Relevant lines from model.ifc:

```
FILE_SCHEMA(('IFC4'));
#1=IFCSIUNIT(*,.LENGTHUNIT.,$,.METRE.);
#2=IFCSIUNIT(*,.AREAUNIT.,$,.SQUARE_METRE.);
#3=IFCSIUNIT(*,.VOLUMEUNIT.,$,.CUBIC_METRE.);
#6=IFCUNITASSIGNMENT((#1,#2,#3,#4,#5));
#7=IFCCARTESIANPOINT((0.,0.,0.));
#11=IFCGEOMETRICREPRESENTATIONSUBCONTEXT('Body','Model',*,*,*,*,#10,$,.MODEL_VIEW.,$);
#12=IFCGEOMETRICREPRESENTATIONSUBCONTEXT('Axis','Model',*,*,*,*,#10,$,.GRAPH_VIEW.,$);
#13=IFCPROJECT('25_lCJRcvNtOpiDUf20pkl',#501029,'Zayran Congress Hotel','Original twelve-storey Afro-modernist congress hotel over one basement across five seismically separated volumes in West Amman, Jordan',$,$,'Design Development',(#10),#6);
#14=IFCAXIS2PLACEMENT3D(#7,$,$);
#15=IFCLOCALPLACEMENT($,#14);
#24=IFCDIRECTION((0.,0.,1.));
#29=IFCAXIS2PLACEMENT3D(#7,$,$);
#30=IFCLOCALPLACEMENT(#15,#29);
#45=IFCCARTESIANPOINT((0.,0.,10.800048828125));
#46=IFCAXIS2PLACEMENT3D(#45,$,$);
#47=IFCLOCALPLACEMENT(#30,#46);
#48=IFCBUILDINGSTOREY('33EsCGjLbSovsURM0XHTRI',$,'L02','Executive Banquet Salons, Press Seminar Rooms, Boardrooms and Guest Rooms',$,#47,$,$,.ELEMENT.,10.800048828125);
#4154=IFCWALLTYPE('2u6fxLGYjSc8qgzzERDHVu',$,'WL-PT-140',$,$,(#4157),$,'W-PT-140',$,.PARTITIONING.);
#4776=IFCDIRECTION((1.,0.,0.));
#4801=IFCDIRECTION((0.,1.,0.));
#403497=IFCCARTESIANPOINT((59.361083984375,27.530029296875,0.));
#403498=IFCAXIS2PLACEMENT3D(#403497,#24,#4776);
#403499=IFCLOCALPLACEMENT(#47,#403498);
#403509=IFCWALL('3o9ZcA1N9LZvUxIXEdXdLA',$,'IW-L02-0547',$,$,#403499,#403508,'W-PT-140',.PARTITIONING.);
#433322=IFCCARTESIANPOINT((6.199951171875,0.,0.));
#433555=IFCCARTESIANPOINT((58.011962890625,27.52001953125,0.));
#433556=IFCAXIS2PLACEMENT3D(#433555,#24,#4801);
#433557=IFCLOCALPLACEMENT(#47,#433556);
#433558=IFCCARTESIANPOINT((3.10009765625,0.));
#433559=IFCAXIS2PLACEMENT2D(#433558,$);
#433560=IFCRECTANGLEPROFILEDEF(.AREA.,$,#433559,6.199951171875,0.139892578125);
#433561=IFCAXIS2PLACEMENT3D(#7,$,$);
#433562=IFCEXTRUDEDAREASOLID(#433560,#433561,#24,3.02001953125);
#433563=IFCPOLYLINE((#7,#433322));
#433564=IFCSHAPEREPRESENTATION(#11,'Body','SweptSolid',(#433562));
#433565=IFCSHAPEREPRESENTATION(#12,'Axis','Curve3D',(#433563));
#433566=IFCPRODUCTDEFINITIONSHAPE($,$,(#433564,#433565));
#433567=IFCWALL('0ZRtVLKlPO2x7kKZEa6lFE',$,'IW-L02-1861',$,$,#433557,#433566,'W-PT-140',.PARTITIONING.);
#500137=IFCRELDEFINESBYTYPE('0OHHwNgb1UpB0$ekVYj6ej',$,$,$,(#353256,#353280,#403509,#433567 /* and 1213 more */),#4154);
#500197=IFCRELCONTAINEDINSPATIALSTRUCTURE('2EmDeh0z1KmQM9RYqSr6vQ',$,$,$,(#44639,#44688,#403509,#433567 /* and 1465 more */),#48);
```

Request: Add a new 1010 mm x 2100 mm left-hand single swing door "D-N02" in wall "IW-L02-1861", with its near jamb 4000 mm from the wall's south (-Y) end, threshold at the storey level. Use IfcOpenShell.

```python
import numpy as np
import ifcopenshell
import ifcopenshell.api.feature
import ifcopenshell.api.geometry
import ifcopenshell.api.root
import ifcopenshell.api.spatial
import ifcopenshell.geom
import ifcopenshell.util.element
import ifcopenshell.util.placement
import ifcopenshell.util.representation
import ifcopenshell.util.shape
import ifcopenshell.util.unit

model = ifcopenshell.open("model.ifc")
unit_scale = ifcopenshell.util.unit.calculate_unit_scale(model)
settings = ifcopenshell.geom.settings()


def volume(element):
    """Net volume in cubic metres, openings subtracted."""
    shape = ifcopenshell.geom.create_shape(settings, element)
    return ifcopenshell.util.shape.get_volume(shape.geometry)


wall = model.by_id(433567)
storey = ifcopenshell.util.element.get_container(wall, ifc_class="IfcBuildingStorey")
context = ifcopenshell.util.representation.get_context(model, "Model", "Body", "MODEL_VIEW")
before = volume(wall)

width, height, from_end, sill = 1.01, 2.1, 4, 0.0  # metres

# The wall runs along its own X axis, and the end named is its -X end.
wall_shape = ifcopenshell.geom.create_shape(settings, wall)
x, y, z = ifcopenshell.util.shape.get_vertices(wall_shape.geometry).T
start = x.min() + from_end
face, thickness = float(y.min()), float(y.max() - y.min())
wall_matrix = ifcopenshell.util.placement.get_local_placement(wall.ObjectPlacement)
level = ifcopenshell.util.placement.get_local_placement(storey.ObjectPlacement)[2, 3]


def in_wall(x, y):
    """Placement at x, y metres in the wall's axes, at sill height."""
    matrix = wall_matrix.copy()
    matrix[:, 3] = wall_matrix @ np.array([x / unit_scale, y / unit_scale, 0.0, 1.0])
    matrix[2, 3] = level + sill / unit_scale
    return matrix


# Opening: a box that overshoots both wall faces by 50 mm.
opening = ifcopenshell.api.root.create_entity(model, ifc_class="IfcOpeningElement", predefined_type="OPENING")
box = ifcopenshell.api.geometry.add_wall_representation(
    model, context=context, length=width, height=height, thickness=thickness + 0.1
)
ifcopenshell.api.geometry.assign_representation(model, product=opening, representation=box)
ifcopenshell.api.geometry.edit_object_placement(model, product=opening, matrix=in_wall(start, face - 0.05), is_si=False)
ifcopenshell.api.feature.add_feature(model, feature=opening, element=wall)

door = ifcopenshell.api.root.create_entity(model, ifc_class="IfcDoor", name="D-N02", predefined_type="DOOR")
door.OverallWidth, door.OverallHeight = width / unit_scale, height / unit_scale
door.OperationType = "SINGLE_SWING_LEFT"
body = ifcopenshell.api.geometry.add_door_representation(
    model,
    context=context,
    overall_width=door.OverallWidth,
    overall_height=door.OverallHeight,
    operation_type="SINGLE_SWING_LEFT",
    lining_properties={"LiningDepth": thickness / unit_scale, "ThresholdDepth": thickness / unit_scale},
)
ifcopenshell.api.geometry.assign_representation(model, product=door, representation=body)
ifcopenshell.api.spatial.assign_container(model, products=[door], relating_structure=storey)
ifcopenshell.api.feature.add_filling(model, opening=opening, element=door)

# The lining spans the wall, so the door starts at the wall face.
ifcopenshell.api.geometry.edit_object_placement(model, product=door, matrix=in_wall(start, face), is_si=False)

after = volume(wall)

print(f"wall volume {before:.3f} -> {after:.3f} m3")

model.write("model_v2.ifc")
```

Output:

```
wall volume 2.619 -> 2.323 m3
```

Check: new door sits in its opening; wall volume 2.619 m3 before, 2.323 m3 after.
